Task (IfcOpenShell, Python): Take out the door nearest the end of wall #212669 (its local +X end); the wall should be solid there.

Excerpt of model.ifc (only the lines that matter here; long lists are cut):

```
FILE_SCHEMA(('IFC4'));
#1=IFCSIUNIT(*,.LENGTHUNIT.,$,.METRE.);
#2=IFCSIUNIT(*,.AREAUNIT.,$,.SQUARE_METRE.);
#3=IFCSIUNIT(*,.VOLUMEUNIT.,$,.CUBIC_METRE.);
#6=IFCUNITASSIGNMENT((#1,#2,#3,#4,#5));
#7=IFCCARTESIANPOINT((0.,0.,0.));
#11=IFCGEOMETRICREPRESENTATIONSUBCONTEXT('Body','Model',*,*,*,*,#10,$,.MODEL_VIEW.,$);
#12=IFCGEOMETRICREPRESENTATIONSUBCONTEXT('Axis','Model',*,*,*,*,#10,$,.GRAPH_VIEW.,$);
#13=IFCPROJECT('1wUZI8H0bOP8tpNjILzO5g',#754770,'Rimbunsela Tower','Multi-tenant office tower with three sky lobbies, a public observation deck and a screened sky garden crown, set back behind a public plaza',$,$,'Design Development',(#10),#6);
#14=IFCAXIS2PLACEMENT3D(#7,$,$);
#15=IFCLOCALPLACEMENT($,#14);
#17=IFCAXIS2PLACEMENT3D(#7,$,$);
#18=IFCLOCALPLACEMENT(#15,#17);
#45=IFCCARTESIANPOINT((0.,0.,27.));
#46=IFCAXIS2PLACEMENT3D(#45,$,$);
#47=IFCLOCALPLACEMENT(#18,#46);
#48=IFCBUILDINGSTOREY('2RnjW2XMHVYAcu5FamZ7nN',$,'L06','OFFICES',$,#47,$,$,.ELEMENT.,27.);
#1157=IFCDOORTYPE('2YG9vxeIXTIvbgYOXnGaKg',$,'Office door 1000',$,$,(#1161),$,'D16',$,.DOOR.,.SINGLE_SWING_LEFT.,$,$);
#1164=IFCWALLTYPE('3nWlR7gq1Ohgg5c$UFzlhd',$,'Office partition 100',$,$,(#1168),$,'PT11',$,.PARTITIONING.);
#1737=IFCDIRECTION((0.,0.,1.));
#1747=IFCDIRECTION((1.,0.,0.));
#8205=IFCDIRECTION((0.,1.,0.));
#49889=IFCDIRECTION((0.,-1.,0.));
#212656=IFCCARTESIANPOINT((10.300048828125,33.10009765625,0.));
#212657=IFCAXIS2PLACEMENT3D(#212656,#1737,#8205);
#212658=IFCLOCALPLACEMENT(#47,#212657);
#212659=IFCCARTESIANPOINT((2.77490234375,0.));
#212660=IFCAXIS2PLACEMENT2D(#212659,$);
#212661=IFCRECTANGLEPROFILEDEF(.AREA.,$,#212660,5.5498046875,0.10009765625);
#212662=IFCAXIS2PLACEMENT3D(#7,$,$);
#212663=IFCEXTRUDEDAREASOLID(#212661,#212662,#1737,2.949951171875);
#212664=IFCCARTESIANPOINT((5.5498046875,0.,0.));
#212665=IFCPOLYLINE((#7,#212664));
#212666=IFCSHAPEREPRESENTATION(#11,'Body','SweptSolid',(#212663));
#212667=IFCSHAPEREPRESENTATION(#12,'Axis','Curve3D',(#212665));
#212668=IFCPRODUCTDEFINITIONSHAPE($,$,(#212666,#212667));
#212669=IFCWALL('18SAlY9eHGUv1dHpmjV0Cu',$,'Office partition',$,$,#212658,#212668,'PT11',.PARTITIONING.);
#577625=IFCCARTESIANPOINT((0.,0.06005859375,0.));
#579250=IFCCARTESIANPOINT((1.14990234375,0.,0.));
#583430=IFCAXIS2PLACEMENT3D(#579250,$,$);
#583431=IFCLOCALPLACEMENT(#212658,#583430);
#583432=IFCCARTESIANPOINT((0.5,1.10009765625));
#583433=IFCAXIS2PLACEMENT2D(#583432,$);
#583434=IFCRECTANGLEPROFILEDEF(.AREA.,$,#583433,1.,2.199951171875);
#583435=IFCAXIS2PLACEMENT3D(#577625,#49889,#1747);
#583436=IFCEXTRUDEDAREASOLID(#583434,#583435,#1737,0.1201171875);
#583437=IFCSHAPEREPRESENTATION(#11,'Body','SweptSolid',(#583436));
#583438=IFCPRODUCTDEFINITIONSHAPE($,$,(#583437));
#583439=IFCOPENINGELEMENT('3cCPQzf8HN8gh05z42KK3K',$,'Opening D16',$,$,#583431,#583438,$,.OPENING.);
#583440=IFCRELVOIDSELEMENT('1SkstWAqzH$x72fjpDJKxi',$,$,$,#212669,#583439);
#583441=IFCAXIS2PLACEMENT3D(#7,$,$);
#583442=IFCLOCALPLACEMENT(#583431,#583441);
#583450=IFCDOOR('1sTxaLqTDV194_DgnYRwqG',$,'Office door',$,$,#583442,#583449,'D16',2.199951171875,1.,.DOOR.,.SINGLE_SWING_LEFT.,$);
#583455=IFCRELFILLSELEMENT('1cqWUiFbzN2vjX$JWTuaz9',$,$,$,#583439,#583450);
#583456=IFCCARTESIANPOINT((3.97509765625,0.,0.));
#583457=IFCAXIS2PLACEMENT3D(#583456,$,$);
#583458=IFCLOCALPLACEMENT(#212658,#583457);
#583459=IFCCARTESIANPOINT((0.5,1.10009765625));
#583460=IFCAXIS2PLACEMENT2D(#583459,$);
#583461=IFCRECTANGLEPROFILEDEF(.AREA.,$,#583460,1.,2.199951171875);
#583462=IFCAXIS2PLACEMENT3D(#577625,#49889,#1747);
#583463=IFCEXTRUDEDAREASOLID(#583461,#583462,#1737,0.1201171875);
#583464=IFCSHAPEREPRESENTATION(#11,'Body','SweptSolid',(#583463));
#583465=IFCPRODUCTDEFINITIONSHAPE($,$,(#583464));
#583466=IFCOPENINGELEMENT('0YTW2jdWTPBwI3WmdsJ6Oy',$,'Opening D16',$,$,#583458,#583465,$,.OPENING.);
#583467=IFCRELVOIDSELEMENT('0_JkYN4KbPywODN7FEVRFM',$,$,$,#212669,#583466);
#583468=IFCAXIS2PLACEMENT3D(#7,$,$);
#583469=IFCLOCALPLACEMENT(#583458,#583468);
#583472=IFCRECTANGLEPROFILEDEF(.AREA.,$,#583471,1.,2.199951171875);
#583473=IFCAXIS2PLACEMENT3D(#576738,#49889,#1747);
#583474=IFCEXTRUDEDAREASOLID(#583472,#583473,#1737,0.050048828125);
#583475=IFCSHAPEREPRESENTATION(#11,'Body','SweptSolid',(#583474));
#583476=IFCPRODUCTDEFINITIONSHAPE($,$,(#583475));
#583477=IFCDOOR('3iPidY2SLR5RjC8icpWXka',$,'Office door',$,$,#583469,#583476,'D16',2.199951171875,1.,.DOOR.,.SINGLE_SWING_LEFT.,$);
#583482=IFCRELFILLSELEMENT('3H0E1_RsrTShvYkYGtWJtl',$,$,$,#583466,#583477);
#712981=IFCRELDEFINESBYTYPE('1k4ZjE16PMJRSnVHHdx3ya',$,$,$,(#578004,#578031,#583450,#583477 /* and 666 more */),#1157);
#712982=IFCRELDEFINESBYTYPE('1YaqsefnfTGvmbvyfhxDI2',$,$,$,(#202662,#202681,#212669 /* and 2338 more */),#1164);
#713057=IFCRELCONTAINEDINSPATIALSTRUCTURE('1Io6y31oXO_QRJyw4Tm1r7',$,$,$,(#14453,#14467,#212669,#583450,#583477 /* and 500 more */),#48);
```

```python
import ifcopenshell
import ifcopenshell.api.feature
import ifcopenshell.api.root
import ifcopenshell.geom
import ifcopenshell.util.shape

model = ifcopenshell.open("model.ifc")
settings = ifcopenshell.geom.settings()


def volume(element):
    """Net volume in cubic metres, openings subtracted."""
    shape = ifcopenshell.geom.create_shape(settings, element)
    return ifcopenshell.util.shape.get_volume(shape.geometry)


door = model.by_guid("3iPidY2SLR5RjC8icpWXka")
opening = door.FillsVoids[0].RelatingOpeningElement
wall = opening.VoidsElements[0].RelatingBuildingElement
before = volume(wall)

ifcopenshell.api.root.remove_product(model, product=door)
ifcopenshell.api.feature.remove_feature(model, feature=opening)

after = volume(wall)

print(f"wall volume {before:.3f} -> {after:.3f} m3")

model.write("model_v2.ifc")
```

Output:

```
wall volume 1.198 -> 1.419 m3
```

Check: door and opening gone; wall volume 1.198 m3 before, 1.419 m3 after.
